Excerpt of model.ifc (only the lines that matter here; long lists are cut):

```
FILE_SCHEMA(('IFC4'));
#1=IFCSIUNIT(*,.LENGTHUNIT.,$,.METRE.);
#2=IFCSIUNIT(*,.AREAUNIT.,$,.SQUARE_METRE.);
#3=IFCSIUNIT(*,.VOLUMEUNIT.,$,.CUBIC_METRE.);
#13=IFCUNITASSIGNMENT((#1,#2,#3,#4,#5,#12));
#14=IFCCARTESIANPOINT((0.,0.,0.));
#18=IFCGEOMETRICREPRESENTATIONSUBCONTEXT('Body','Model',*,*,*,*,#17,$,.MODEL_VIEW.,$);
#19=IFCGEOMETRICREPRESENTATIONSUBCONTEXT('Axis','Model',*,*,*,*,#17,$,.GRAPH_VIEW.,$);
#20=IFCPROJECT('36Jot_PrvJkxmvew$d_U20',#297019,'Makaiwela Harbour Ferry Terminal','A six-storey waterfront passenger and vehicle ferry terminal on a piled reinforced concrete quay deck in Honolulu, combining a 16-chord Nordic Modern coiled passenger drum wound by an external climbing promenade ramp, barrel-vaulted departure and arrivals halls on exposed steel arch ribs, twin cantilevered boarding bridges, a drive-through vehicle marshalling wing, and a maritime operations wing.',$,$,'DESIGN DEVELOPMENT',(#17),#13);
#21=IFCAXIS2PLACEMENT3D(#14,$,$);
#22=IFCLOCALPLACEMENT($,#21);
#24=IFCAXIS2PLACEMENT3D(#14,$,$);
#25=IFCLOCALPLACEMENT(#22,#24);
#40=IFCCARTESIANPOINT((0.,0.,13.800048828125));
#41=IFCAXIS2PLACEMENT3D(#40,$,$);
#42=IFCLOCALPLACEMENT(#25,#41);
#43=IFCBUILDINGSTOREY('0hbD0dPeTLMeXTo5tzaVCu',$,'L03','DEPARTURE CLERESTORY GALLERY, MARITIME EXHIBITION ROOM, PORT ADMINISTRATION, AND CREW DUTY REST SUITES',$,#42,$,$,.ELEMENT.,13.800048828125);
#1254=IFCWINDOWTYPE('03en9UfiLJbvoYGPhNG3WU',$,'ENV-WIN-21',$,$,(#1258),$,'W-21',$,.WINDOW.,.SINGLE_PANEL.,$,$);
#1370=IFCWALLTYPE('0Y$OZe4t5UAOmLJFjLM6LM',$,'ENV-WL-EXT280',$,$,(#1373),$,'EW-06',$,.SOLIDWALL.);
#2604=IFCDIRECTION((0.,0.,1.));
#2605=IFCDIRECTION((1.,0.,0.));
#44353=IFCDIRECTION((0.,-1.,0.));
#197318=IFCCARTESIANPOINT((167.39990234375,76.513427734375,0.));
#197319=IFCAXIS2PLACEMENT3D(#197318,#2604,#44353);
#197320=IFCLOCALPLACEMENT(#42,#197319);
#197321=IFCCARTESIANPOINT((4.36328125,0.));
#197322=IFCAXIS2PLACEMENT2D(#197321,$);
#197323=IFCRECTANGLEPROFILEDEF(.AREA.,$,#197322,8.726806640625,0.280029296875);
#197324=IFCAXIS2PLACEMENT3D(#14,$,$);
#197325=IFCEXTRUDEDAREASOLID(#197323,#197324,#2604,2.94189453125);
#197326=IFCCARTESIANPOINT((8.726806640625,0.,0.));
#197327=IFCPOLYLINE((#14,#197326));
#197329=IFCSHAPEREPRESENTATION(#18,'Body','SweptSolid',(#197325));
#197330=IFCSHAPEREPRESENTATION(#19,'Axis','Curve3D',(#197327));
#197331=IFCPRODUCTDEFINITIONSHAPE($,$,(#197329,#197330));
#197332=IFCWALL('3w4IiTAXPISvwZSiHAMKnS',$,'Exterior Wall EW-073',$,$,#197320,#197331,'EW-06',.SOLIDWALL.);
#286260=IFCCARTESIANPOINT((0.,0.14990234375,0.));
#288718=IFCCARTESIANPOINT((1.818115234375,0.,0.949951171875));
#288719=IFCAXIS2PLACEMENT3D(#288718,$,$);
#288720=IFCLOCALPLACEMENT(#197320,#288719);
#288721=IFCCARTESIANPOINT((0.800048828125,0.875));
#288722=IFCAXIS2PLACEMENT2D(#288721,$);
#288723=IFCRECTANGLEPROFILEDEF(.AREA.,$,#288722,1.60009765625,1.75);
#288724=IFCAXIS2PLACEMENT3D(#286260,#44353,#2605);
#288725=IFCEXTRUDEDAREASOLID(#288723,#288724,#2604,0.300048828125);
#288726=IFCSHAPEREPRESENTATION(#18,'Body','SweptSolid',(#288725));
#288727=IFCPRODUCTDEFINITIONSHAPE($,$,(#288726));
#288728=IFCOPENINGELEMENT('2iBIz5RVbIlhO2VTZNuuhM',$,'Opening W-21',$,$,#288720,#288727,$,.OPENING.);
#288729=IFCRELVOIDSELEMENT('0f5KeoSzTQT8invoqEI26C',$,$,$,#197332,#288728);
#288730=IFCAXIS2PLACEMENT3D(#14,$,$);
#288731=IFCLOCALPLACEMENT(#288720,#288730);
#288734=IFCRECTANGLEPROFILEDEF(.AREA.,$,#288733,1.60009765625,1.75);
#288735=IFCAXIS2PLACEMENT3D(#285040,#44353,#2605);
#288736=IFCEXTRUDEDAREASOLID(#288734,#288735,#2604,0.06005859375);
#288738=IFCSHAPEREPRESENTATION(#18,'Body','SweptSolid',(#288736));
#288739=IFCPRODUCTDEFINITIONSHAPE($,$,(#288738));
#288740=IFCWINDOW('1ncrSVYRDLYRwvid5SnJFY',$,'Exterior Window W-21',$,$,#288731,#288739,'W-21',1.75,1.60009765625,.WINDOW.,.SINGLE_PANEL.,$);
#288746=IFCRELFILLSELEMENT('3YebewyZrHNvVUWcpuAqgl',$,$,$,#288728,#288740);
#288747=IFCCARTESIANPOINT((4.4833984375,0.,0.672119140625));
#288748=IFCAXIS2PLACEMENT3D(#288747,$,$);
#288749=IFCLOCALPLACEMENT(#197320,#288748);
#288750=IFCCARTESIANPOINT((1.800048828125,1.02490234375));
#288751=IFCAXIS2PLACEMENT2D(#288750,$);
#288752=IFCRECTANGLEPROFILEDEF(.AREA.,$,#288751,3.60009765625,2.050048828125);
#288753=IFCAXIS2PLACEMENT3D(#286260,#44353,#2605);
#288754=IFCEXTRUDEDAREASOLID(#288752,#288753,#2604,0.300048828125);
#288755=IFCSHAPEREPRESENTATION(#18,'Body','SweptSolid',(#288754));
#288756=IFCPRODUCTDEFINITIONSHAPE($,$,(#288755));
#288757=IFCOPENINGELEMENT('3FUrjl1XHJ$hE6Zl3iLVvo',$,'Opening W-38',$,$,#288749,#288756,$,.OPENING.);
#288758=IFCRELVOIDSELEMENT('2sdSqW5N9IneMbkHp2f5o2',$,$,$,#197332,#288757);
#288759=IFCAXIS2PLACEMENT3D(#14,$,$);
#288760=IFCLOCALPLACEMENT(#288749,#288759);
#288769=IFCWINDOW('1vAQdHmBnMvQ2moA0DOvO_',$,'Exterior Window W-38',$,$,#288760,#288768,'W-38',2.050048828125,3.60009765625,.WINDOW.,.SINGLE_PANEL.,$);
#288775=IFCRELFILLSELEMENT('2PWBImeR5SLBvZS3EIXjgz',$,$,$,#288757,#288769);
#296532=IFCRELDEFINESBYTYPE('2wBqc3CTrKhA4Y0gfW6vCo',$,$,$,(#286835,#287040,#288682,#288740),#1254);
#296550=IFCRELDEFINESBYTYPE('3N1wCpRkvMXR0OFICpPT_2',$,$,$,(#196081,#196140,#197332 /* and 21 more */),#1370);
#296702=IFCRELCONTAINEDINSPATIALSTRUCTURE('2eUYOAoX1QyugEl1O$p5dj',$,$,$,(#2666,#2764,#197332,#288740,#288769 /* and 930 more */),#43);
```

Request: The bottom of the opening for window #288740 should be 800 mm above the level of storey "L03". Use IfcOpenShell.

```python
import numpy as np
import ifcopenshell
import ifcopenshell.api.geometry
import ifcopenshell.geom
import ifcopenshell.util.element
import ifcopenshell.util.placement
import ifcopenshell.util.shape
import ifcopenshell.util.unit

model = ifcopenshell.open("model.ifc")
unit_scale = ifcopenshell.util.unit.calculate_unit_scale(model)

window = model.by_guid("1ncrSVYRDLYRwvid5SnJFY")
opening = window.FillsVoids[0].RelatingOpeningElement
storey = ifcopenshell.util.element.get_container(window, ifc_class="IfcBuildingStorey")
level = ifcopenshell.util.placement.get_local_placement(storey.ObjectPlacement)[2, 3]

# The opening's origin need not be at the sill, so measure its lowest point.
shape = ifcopenshell.geom.create_shape(ifcopenshell.geom.settings(), opening)
bottom = ifcopenshell.util.shape.get_shape_bottom_elevation(shape, shape.geometry) / unit_scale
dz = level + 0.8 / unit_scale - bottom

shift = np.array([0.0, 0.0, dz])
# The window is placed relative to its opening, so it follows when the opening moves.
matrix = ifcopenshell.util.placement.get_local_placement(opening.ObjectPlacement)
matrix[:3, 3] += shift
ifcopenshell.api.geometry.edit_object_placement(
    model, product=opening, matrix=matrix, is_si=False, should_transform_children=True
)

print(f"moved by {dz * unit_scale:+.3f} m")

model.write("model_v2.ifc")
```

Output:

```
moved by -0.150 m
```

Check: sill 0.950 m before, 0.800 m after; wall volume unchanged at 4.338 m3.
